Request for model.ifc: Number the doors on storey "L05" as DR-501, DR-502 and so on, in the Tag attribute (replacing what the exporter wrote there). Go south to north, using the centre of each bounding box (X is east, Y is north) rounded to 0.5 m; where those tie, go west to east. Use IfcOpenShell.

First a look at what the model holds.

```python
import ifcopenshell
import ifcopenshell.util.element
import ifcopenshell.util.placement

model = ifcopenshell.open("model.ifc")
print(model.schema)
storey = next(s for s in model.by_type("IfcBuildingStorey") if s.Name == "L05")
doors = [e for e in ifcopenshell.util.element.get_decomposition(storey) if e.is_a("IfcDoor")]
for e in sorted(doors, key=lambda e: e.id()):
    origin = ifcopenshell.util.placement.get_local_placement(e.ObjectPlacement)[:3, 3]
    print(e.id(), e.Tag, e.Name, origin.round(2) + 0.0, sep=" | ")
```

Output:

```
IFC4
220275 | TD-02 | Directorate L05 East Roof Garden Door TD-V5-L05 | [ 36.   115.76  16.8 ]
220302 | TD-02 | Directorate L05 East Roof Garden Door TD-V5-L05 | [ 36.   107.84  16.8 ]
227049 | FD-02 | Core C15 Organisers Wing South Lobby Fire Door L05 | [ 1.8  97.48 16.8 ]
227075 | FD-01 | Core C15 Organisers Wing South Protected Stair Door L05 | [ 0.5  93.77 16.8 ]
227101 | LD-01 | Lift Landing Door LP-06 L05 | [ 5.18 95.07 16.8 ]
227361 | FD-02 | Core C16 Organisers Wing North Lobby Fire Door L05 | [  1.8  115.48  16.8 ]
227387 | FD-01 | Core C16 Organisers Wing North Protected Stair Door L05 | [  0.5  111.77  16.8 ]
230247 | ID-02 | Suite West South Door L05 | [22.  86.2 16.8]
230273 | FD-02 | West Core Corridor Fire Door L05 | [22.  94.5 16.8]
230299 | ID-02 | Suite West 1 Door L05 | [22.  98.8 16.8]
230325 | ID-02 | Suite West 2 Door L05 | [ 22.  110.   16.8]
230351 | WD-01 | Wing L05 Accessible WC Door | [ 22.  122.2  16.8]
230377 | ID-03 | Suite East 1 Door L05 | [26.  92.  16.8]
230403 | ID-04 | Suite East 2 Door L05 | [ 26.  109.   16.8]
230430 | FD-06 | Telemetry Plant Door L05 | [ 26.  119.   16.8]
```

```python
import ifcopenshell
import ifcopenshell.geom
import ifcopenshell.util.element
import ifcopenshell.util.shape

model = ifcopenshell.open("model.ifc")
settings = ifcopenshell.geom.settings()
settings.set("use-world-coords", True)


def centre(element):
    shape = ifcopenshell.geom.create_shape(settings, element)
    return ifcopenshell.util.shape.get_bbox_centroid(shape.geometry)


storey = next(s for s in model.by_type("IfcBuildingStorey") if s.Name == "L05")
doors = [e for e in ifcopenshell.util.element.get_decomposition(storey) if e.is_a("IfcDoor")]

# Insertion points can sit at a corner or the storey origin, so sort by the geometry (in metres).
centres = {e: centre(e) for e in doors}
doors.sort(key=lambda e: (round(centres[e][1] / 0.5), centres[e][0]))

for i, e in enumerate(doors, start=1):
    number = f"DR-5{i:02d}"
    e.Tag = number
    print(e.id(), number)

model.write("model_rev.ifc")
```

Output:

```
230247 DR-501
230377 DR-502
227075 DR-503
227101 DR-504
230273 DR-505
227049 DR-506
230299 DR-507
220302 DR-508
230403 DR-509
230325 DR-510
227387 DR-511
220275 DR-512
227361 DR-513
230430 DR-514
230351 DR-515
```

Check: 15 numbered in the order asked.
